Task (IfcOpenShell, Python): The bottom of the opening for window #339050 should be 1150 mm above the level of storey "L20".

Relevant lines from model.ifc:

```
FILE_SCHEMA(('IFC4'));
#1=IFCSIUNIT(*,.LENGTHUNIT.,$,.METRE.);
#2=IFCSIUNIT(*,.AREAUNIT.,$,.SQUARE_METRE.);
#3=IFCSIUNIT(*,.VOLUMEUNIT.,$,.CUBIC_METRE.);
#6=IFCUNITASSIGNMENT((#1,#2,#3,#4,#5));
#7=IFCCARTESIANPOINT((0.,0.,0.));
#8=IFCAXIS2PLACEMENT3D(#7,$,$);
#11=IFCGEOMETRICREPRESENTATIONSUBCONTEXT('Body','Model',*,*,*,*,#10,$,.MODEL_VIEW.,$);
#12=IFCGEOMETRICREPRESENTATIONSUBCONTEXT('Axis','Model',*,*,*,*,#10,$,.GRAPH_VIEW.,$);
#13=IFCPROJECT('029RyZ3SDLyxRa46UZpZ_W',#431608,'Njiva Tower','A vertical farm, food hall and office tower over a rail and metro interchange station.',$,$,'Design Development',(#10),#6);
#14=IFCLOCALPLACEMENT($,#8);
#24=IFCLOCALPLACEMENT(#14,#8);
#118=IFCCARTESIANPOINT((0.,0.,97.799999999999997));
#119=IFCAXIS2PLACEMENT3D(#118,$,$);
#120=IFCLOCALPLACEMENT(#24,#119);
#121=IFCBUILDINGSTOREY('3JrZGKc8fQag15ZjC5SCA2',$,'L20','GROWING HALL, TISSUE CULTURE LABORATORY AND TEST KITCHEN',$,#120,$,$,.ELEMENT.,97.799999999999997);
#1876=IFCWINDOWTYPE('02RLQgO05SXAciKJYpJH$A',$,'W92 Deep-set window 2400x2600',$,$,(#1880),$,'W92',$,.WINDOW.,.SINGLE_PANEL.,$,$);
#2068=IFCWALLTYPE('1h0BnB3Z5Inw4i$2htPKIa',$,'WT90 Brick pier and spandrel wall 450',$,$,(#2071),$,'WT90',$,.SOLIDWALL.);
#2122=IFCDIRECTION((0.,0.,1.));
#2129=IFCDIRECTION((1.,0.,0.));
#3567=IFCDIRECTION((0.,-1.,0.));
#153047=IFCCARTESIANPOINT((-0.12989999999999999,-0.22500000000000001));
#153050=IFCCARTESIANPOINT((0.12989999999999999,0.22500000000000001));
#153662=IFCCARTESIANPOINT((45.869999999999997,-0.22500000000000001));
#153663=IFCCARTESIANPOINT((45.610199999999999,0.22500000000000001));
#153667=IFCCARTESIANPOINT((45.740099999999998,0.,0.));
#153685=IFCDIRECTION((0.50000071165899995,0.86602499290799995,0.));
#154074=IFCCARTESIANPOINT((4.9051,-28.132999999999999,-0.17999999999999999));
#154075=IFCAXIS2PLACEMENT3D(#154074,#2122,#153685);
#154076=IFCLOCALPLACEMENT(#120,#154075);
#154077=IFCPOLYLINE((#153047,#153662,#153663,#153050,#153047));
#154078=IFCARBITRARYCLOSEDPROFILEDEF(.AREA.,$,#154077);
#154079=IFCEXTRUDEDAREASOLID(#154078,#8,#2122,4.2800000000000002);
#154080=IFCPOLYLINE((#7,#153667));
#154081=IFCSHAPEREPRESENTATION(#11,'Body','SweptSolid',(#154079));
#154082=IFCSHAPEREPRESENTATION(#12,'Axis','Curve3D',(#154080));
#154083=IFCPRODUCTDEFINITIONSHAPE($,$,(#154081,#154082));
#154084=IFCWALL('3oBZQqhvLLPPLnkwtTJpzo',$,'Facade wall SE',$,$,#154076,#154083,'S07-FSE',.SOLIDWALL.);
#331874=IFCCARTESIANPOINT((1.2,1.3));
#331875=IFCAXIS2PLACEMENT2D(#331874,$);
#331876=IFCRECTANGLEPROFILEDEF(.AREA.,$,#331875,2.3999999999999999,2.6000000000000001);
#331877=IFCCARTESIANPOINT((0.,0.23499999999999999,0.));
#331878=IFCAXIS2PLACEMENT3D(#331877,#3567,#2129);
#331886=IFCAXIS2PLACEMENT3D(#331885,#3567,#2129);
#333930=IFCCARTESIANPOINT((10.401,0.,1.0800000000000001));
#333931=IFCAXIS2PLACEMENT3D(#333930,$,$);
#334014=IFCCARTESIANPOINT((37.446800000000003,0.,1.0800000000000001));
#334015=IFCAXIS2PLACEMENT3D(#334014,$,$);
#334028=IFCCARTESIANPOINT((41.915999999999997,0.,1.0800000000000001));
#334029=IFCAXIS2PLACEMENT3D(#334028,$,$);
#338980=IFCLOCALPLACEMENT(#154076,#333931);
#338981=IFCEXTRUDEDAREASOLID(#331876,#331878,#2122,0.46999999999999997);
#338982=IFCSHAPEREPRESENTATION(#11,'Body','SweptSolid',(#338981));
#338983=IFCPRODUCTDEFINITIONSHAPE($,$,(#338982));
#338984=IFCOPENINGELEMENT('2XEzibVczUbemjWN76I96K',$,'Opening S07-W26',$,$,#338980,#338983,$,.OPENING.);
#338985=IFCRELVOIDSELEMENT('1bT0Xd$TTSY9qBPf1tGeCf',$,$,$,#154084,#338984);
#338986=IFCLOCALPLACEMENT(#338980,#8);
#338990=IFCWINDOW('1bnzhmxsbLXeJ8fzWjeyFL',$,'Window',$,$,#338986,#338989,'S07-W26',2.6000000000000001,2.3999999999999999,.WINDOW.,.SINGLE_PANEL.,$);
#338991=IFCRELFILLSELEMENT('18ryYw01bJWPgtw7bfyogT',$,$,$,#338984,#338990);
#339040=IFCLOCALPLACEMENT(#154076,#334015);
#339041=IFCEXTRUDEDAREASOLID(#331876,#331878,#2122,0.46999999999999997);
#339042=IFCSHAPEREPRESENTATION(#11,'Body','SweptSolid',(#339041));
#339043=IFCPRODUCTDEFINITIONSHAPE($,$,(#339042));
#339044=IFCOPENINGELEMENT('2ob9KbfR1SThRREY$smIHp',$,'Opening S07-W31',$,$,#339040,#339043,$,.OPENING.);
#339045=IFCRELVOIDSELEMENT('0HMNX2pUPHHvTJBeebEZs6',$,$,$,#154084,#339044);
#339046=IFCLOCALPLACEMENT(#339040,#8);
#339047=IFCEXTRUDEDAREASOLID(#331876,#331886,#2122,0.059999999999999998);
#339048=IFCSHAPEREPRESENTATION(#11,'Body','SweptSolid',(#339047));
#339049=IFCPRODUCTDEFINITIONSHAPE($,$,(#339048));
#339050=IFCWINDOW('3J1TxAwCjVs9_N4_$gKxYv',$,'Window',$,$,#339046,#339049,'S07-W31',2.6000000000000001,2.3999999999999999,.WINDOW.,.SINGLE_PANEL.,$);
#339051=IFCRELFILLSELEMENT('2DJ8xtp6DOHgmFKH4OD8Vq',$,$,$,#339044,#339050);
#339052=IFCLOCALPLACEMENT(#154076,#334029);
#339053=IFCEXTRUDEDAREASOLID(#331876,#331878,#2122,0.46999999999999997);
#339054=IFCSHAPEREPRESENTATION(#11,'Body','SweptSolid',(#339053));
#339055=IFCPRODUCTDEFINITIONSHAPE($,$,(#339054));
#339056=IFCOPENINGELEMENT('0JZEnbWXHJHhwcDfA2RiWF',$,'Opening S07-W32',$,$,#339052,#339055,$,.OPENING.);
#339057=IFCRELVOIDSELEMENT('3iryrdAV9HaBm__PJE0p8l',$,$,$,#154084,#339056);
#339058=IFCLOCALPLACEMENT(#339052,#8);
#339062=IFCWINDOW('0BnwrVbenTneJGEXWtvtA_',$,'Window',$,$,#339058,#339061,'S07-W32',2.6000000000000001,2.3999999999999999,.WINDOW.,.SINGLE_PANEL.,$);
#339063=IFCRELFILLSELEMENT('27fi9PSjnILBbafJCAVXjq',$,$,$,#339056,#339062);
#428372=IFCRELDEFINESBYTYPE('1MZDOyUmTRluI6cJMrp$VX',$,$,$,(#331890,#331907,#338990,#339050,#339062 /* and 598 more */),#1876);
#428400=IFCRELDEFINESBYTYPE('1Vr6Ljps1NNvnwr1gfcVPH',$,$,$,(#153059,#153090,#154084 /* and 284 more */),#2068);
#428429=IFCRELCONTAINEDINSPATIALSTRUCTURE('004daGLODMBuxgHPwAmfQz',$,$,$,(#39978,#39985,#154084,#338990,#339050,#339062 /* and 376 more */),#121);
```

```python
import numpy as np
import ifcopenshell
import ifcopenshell.api.geometry
import ifcopenshell.geom
import ifcopenshell.util.element
import ifcopenshell.util.placement
import ifcopenshell.util.shape
import ifcopenshell.util.unit

model = ifcopenshell.open("model.ifc")
unit_scale = ifcopenshell.util.unit.calculate_unit_scale(model)

window = model.by_guid("3J1TxAwCjVs9_N4_$gKxYv")
opening = window.FillsVoids[0].RelatingOpeningElement
storey = ifcopenshell.util.element.get_container(window, ifc_class="IfcBuildingStorey")
level = ifcopenshell.util.placement.get_local_placement(storey.ObjectPlacement)[2, 3]

# The opening's origin need not be at the sill, so measure its lowest point.
shape = ifcopenshell.geom.create_shape(ifcopenshell.geom.settings(), opening)
bottom = ifcopenshell.util.shape.get_shape_bottom_elevation(shape, shape.geometry) / unit_scale
dz = level + 1.15 / unit_scale - bottom

shift = np.array([0.0, 0.0, dz])
# The window is placed relative to its opening, so it follows when the opening moves.
matrix = ifcopenshell.util.placement.get_local_placement(opening.ObjectPlacement)
matrix[:3, 3] += shift
ifcopenshell.api.geometry.edit_object_placement(
    model, product=opening, matrix=matrix, is_si=False, should_transform_children=True
)

print(f"moved by {dz * unit_scale:+.3f} m")

model.write("model_v2.ifc")
```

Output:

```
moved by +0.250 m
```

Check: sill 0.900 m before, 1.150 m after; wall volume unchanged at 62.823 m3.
